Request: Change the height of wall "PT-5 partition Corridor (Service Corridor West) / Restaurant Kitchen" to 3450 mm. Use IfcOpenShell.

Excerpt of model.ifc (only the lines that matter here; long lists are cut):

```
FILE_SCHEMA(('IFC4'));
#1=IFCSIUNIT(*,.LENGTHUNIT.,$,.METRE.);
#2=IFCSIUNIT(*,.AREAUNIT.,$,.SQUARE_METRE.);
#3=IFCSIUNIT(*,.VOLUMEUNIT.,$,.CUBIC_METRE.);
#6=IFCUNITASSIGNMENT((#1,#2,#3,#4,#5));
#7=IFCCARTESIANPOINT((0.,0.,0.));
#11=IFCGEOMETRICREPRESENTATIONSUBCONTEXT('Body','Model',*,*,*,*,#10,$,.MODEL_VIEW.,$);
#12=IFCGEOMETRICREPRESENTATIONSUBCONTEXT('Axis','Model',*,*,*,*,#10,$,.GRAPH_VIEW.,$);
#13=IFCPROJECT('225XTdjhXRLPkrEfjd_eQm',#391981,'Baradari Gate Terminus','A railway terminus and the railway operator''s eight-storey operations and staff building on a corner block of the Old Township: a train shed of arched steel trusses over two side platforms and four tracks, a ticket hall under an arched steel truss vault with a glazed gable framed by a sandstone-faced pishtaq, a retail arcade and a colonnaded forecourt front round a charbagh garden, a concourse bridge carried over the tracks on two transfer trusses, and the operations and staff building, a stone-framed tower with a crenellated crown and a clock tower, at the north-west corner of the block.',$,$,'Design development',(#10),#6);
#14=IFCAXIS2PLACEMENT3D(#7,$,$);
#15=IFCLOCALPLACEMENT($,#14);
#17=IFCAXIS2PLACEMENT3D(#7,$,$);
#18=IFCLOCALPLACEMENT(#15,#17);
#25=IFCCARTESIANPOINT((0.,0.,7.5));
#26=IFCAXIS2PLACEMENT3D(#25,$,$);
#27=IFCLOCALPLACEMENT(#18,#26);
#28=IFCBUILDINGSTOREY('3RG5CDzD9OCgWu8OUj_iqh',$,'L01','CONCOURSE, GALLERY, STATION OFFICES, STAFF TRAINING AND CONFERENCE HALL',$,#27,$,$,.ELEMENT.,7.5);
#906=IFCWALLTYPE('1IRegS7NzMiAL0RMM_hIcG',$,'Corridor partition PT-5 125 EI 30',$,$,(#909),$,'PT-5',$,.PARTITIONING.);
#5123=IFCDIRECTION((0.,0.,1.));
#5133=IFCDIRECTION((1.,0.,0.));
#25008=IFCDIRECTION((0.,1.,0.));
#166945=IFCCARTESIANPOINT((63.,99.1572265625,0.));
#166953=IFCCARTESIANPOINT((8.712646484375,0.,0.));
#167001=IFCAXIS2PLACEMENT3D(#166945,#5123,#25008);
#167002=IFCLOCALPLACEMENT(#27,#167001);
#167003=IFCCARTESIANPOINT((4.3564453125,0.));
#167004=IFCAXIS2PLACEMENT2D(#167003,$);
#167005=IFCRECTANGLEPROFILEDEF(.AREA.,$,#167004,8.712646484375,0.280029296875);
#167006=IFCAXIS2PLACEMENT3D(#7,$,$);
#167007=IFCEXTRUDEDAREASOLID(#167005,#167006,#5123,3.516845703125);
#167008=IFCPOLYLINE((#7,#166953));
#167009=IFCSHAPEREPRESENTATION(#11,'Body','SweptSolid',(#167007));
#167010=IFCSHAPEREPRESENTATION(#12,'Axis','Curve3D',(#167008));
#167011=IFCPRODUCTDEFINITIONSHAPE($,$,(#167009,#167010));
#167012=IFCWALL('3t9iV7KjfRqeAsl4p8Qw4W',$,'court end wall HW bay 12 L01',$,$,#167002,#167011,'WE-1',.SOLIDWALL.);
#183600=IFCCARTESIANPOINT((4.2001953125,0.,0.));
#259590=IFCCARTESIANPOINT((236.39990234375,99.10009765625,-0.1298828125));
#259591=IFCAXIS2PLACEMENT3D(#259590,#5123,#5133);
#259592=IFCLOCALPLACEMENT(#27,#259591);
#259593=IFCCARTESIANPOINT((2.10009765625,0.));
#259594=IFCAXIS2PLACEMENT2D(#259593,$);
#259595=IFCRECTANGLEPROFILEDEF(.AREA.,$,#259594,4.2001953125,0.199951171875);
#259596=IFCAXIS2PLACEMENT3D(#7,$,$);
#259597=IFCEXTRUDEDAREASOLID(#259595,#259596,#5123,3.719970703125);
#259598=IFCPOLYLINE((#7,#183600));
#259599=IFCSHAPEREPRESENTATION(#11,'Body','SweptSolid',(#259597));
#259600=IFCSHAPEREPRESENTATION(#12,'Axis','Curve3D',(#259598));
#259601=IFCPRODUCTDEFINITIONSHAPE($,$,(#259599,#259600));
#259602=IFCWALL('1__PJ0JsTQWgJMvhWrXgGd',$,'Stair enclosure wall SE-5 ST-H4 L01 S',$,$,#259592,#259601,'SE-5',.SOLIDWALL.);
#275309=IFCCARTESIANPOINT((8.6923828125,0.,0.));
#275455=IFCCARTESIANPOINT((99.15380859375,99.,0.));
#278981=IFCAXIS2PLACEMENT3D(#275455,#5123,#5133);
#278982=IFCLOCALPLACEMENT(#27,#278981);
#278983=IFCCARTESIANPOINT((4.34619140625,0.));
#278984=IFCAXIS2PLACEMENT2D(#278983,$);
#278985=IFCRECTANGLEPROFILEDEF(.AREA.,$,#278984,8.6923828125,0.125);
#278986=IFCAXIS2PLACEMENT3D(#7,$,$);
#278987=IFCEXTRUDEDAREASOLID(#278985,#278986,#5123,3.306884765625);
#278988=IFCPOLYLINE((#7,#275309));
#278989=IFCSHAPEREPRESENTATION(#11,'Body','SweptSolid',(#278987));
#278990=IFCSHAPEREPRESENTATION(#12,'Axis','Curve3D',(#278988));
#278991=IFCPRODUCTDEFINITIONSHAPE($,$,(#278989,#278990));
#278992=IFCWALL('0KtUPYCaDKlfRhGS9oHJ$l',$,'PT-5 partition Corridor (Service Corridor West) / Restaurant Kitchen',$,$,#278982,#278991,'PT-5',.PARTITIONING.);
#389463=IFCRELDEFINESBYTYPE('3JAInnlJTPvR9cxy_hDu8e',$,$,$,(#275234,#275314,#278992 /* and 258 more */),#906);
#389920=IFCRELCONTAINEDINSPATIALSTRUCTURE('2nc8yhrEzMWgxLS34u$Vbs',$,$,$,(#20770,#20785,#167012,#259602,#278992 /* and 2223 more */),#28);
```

```python
import ifcopenshell
import ifcopenshell.geom
import ifcopenshell.util.representation
import ifcopenshell.util.shape

model = ifcopenshell.open("model.ifc")
settings = ifcopenshell.geom.settings()


def volume(element):
    """Net volume in cubic metres, openings subtracted."""
    shape = ifcopenshell.geom.create_shape(settings, element)
    return ifcopenshell.util.shape.get_volume(shape.geometry)


wall = model.by_id(278992)
before = volume(wall)

body = ifcopenshell.util.representation.get_representation(wall, "Model", "Body")
solid = body.Items[0]
old_height = solid.Depth
solid.Depth = 3.45
after = volume(wall)

print(f"height {old_height:g} -> {solid.Depth:g}, volume {before:.3f} -> {after:.3f} m3")

model.write("model_rev.ifc")
```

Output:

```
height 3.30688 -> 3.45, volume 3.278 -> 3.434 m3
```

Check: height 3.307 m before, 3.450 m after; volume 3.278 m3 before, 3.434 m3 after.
